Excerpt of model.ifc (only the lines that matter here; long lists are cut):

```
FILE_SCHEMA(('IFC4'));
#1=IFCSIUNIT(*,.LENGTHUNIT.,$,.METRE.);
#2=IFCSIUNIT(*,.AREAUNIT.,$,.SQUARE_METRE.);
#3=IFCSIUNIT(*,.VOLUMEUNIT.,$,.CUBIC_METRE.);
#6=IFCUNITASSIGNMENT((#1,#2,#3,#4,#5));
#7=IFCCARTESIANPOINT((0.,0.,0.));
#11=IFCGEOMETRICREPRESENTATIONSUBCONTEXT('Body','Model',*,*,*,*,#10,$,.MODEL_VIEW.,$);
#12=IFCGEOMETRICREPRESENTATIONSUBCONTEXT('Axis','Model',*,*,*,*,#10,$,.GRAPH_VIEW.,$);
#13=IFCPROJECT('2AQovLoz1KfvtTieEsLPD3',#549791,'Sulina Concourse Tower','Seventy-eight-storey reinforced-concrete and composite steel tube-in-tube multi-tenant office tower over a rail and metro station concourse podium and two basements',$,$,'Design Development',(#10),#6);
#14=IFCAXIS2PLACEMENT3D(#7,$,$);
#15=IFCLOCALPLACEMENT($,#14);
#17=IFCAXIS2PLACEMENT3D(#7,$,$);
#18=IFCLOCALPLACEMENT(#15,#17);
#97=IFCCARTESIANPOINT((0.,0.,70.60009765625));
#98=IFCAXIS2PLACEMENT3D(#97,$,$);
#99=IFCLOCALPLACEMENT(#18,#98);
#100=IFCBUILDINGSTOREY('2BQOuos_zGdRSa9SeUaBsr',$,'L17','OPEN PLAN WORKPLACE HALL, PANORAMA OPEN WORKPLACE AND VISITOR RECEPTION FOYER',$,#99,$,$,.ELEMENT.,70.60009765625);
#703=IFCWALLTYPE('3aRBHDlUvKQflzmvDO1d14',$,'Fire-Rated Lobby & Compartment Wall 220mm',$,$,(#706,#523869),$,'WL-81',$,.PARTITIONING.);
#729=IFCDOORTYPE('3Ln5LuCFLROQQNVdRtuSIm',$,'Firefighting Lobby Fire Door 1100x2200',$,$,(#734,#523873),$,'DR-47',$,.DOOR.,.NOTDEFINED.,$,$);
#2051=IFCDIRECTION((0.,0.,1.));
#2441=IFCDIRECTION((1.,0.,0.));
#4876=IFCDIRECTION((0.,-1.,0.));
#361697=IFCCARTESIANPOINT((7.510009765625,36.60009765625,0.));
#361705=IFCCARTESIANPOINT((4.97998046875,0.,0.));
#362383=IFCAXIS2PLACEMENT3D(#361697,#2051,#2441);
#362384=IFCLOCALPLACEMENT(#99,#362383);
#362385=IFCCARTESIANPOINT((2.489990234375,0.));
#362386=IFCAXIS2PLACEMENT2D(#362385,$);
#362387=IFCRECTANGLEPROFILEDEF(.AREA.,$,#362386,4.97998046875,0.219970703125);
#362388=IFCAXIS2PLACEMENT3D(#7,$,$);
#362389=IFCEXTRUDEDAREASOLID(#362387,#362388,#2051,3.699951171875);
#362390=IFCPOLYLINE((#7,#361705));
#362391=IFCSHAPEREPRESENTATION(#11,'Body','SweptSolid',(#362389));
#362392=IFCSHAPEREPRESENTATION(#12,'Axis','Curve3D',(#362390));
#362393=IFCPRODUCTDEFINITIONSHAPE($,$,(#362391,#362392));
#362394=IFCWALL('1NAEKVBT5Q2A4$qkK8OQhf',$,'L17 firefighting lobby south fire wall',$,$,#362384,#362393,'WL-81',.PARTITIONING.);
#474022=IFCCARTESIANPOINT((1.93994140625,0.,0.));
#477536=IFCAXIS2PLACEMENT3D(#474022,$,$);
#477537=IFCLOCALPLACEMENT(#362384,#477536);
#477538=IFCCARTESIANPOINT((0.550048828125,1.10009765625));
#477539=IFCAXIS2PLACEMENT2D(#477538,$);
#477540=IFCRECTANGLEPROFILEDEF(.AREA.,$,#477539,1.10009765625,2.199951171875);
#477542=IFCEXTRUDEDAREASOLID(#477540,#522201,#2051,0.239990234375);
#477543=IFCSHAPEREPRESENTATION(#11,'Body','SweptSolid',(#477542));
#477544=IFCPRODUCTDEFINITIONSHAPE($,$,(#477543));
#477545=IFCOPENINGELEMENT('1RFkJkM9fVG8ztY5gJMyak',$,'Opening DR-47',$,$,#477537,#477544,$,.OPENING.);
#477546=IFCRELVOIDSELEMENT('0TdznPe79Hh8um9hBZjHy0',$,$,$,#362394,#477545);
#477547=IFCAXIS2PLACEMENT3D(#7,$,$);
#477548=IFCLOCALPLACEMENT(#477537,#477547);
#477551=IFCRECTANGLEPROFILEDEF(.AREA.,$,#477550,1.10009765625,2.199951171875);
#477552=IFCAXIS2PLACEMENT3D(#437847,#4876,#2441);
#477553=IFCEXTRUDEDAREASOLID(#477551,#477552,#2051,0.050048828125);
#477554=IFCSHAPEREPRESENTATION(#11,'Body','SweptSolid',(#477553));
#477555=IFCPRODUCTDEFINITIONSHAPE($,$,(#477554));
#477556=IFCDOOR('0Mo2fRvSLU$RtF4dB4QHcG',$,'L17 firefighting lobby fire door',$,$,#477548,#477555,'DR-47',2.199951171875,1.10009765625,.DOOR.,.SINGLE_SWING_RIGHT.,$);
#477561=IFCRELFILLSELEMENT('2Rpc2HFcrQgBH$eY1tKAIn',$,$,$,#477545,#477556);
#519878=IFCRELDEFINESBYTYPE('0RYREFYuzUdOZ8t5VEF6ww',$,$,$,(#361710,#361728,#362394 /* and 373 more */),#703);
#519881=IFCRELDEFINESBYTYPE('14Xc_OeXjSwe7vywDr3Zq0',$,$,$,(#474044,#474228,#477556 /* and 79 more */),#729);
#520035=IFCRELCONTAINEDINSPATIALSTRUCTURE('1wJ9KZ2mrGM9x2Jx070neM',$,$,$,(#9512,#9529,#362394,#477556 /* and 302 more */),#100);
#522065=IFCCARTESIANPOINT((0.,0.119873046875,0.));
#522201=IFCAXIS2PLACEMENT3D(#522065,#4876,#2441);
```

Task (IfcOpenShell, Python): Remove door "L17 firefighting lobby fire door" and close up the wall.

```python
import ifcopenshell
import ifcopenshell.api.feature
import ifcopenshell.api.root
import ifcopenshell.geom
import ifcopenshell.util.shape

model = ifcopenshell.open("model.ifc")
settings = ifcopenshell.geom.settings()


def volume(element):
    """Net volume in cubic metres, openings subtracted."""
    shape = ifcopenshell.geom.create_shape(settings, element)
    return ifcopenshell.util.shape.get_volume(shape.geometry)


door = model.by_guid("0Mo2fRvSLU$RtF4dB4QHcG")
opening = door.FillsVoids[0].RelatingOpeningElement
wall = opening.VoidsElements[0].RelatingBuildingElement
before = volume(wall)

ifcopenshell.api.root.remove_product(model, product=door)
ifcopenshell.api.feature.remove_feature(model, feature=opening)

after = volume(wall)

print(f"wall volume {before:.3f} -> {after:.3f} m3")

model.write("model-out.ifc")
```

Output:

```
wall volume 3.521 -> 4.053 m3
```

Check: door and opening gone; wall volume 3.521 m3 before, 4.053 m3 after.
